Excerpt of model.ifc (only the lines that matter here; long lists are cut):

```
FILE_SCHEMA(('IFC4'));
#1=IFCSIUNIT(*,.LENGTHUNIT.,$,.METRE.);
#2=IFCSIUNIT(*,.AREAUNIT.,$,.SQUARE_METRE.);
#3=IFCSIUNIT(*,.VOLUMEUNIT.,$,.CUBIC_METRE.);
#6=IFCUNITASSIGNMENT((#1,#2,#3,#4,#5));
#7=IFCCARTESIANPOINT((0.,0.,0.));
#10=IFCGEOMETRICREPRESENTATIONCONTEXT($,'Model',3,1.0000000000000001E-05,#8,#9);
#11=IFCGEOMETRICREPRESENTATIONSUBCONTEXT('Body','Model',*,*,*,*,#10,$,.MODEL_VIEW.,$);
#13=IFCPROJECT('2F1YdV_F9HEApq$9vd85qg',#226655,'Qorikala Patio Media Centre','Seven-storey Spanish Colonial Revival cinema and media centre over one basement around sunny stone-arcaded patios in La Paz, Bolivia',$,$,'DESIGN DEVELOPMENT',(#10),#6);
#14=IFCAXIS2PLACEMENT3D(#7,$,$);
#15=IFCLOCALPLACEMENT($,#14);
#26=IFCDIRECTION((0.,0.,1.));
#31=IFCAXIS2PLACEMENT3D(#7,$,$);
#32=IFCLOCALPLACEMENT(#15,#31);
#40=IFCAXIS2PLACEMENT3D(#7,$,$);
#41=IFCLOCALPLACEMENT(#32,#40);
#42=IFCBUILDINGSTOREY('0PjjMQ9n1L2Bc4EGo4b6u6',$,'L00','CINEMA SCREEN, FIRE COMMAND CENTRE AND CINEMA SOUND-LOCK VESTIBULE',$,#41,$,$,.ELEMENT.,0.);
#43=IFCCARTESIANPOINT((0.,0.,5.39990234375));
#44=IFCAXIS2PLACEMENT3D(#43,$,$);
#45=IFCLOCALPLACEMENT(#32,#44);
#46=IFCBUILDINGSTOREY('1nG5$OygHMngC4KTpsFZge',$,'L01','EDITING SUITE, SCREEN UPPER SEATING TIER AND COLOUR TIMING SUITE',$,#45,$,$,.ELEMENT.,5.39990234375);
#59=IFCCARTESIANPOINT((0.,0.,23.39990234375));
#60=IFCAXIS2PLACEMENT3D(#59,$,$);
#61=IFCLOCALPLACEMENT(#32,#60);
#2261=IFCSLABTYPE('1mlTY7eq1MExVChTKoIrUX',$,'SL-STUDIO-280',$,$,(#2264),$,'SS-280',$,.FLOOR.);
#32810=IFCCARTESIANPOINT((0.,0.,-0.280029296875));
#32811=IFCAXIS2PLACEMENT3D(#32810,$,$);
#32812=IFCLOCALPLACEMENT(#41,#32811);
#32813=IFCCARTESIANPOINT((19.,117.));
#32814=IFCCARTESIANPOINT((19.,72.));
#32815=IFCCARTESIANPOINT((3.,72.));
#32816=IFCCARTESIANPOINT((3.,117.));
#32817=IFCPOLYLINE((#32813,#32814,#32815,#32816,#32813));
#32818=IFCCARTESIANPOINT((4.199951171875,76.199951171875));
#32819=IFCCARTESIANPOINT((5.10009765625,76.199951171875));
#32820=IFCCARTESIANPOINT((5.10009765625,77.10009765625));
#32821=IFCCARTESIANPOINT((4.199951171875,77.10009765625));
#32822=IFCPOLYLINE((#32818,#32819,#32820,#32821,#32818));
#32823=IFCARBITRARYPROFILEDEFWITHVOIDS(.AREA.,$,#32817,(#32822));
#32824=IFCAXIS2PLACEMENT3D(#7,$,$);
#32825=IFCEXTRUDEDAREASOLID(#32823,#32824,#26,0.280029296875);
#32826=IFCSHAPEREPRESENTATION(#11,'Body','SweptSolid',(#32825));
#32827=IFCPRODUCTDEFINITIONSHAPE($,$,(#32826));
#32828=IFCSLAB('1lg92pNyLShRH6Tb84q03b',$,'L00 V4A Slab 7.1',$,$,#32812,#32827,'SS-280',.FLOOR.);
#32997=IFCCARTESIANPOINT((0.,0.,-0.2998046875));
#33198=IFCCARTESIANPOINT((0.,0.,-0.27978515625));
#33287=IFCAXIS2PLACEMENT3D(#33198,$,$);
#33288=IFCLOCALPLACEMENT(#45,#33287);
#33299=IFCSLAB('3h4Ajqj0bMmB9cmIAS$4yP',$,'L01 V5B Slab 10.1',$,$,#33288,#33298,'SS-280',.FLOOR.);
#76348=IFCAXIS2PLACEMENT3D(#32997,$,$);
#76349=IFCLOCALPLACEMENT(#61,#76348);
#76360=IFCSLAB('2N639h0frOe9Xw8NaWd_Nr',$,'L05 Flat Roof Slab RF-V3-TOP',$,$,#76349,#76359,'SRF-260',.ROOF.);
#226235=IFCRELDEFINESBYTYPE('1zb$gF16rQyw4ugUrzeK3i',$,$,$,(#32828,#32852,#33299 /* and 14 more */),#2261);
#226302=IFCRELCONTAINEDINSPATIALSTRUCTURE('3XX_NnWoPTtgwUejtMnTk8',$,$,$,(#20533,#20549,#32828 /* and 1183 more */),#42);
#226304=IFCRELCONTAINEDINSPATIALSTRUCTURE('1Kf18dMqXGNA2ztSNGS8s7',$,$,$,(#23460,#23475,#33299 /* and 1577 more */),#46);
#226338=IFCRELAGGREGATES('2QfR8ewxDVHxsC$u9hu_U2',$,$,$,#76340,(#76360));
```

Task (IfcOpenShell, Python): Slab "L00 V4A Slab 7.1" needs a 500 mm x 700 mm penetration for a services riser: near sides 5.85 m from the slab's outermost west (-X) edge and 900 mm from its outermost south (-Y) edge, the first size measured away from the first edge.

```python
import numpy as np
import ifcopenshell
import ifcopenshell.api.feature
import ifcopenshell.api.geometry
import ifcopenshell.api.root
import ifcopenshell.geom
import ifcopenshell.util.placement
import ifcopenshell.util.representation
import ifcopenshell.util.shape
import ifcopenshell.util.unit

model = ifcopenshell.open("model.ifc")
unit_scale = ifcopenshell.util.unit.calculate_unit_scale(model)
settings = ifcopenshell.geom.settings()


def volume(element):
    """Net volume in cubic metres, openings subtracted."""
    shape = ifcopenshell.geom.create_shape(settings, element)
    return ifcopenshell.util.shape.get_volume(shape.geometry)


slab = model.by_guid("1lg92pNyLShRH6Tb84q03b")
before = volume(slab)

# Extent in the slab's own axes, in metres. The edges named are its -X and -Y sides.
slab_shape = ifcopenshell.geom.create_shape(settings, slab)
vertices = ifcopenshell.util.shape.get_vertices(slab_shape.geometry)
x_min, y_min, bottom = vertices.min(axis=0)
top = vertices[:, 2].max()

opening = ifcopenshell.api.root.create_entity(model, ifc_class="IfcOpeningElement", name="Services riser opening", predefined_type="OPENING")
context = ifcopenshell.util.representation.get_context(model, "Model", "Body", "MODEL_VIEW")
width, depth = 0.5, 0.7
outline = [(0.0, 0.0), (width, 0.0), (width, depth), (0.0, depth), (0.0, 0.0)]
# Overshoot both faces by 50 mm so the cut is clean.
shape = ifcopenshell.api.geometry.add_slab_representation(
    model, context=context, depth=top - bottom + 0.1, polyline=outline
)
ifcopenshell.api.geometry.assign_representation(model, product=opening, representation=shape)

matrix = ifcopenshell.util.placement.get_local_placement(slab.ObjectPlacement)
matrix[:, 3] = matrix @ np.append(np.array([x_min + 5.85, y_min + 0.9, bottom - 0.05]) / unit_scale, 1.0)
ifcopenshell.api.geometry.edit_object_placement(model, product=opening, matrix=matrix, is_si=False)
ifcopenshell.api.feature.add_feature(model, feature=opening, element=slab)

after = volume(slab)

print(f"slab volume {before:.3f} -> {after:.3f} m3")

model.write("model_v2.ifc")
```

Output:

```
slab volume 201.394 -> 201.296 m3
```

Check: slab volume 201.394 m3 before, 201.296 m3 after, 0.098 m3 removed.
